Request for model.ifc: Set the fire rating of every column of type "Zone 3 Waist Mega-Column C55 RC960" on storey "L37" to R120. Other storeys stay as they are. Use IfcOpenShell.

First a look at what the model holds.

```python
import ifcopenshell
import ifcopenshell.util.element

model = ifcopenshell.open("model.ifc")
print(model.schema)
storey = next(s for s in model.by_type("IfcBuildingStorey") if s.Name == "L37")
columns = [e for e in ifcopenshell.util.element.get_decomposition(storey) if e.is_a("IfcColumn")]
seen = {}
for e in columns:
    element_type = ifcopenshell.util.element.get_type(e)
    key = (element_type.Name if element_type != e and element_type else None, ifcopenshell.util.element.get_pset(e, "Pset_ColumnCommon", "FireRating"))
    seen[key] = seen.get(key, 0) + 1
for (name, value), count in sorted(seen.items(), key=str):
    print(count, "x", name, "|", value)
```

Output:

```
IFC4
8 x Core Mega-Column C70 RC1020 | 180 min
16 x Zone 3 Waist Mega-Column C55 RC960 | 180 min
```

```python
import ifcopenshell
import ifcopenshell.api.pset
import ifcopenshell.util.element

model = ifcopenshell.open("model.ifc")

storey = next(s for s in model.by_type("IfcBuildingStorey") if s.Name == "L37")
columns = [e for e in ifcopenshell.util.element.get_decomposition(storey) if e.is_a("IfcColumn")]

count = 0
for e in columns:
    element_type = ifcopenshell.util.element.get_type(e)
    if element_type in (None, e) or element_type.Name != "Zone 3 Waist Mega-Column C55 RC960":
        continue
    found = ifcopenshell.util.element.get_pset(e, "Pset_ColumnCommon", should_inherit=False)
    if found:
        pset = model.by_id(found["id"])
        if len(ifcopenshell.util.element.get_elements_by_pset(pset)) > 1:
            pset = ifcopenshell.api.pset.unshare_pset(model, products=[e], pset=pset)[0]
    else:
        pset = ifcopenshell.api.pset.add_pset(model, product=e, name="Pset_ColumnCommon")
    ifcopenshell.api.pset.edit_pset(model, pset=pset, properties={"FireRating": "R120"})
    count += 1

print(count, "columns updated")

model.write("model_rev.ifc")
```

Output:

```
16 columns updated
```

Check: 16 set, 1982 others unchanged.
